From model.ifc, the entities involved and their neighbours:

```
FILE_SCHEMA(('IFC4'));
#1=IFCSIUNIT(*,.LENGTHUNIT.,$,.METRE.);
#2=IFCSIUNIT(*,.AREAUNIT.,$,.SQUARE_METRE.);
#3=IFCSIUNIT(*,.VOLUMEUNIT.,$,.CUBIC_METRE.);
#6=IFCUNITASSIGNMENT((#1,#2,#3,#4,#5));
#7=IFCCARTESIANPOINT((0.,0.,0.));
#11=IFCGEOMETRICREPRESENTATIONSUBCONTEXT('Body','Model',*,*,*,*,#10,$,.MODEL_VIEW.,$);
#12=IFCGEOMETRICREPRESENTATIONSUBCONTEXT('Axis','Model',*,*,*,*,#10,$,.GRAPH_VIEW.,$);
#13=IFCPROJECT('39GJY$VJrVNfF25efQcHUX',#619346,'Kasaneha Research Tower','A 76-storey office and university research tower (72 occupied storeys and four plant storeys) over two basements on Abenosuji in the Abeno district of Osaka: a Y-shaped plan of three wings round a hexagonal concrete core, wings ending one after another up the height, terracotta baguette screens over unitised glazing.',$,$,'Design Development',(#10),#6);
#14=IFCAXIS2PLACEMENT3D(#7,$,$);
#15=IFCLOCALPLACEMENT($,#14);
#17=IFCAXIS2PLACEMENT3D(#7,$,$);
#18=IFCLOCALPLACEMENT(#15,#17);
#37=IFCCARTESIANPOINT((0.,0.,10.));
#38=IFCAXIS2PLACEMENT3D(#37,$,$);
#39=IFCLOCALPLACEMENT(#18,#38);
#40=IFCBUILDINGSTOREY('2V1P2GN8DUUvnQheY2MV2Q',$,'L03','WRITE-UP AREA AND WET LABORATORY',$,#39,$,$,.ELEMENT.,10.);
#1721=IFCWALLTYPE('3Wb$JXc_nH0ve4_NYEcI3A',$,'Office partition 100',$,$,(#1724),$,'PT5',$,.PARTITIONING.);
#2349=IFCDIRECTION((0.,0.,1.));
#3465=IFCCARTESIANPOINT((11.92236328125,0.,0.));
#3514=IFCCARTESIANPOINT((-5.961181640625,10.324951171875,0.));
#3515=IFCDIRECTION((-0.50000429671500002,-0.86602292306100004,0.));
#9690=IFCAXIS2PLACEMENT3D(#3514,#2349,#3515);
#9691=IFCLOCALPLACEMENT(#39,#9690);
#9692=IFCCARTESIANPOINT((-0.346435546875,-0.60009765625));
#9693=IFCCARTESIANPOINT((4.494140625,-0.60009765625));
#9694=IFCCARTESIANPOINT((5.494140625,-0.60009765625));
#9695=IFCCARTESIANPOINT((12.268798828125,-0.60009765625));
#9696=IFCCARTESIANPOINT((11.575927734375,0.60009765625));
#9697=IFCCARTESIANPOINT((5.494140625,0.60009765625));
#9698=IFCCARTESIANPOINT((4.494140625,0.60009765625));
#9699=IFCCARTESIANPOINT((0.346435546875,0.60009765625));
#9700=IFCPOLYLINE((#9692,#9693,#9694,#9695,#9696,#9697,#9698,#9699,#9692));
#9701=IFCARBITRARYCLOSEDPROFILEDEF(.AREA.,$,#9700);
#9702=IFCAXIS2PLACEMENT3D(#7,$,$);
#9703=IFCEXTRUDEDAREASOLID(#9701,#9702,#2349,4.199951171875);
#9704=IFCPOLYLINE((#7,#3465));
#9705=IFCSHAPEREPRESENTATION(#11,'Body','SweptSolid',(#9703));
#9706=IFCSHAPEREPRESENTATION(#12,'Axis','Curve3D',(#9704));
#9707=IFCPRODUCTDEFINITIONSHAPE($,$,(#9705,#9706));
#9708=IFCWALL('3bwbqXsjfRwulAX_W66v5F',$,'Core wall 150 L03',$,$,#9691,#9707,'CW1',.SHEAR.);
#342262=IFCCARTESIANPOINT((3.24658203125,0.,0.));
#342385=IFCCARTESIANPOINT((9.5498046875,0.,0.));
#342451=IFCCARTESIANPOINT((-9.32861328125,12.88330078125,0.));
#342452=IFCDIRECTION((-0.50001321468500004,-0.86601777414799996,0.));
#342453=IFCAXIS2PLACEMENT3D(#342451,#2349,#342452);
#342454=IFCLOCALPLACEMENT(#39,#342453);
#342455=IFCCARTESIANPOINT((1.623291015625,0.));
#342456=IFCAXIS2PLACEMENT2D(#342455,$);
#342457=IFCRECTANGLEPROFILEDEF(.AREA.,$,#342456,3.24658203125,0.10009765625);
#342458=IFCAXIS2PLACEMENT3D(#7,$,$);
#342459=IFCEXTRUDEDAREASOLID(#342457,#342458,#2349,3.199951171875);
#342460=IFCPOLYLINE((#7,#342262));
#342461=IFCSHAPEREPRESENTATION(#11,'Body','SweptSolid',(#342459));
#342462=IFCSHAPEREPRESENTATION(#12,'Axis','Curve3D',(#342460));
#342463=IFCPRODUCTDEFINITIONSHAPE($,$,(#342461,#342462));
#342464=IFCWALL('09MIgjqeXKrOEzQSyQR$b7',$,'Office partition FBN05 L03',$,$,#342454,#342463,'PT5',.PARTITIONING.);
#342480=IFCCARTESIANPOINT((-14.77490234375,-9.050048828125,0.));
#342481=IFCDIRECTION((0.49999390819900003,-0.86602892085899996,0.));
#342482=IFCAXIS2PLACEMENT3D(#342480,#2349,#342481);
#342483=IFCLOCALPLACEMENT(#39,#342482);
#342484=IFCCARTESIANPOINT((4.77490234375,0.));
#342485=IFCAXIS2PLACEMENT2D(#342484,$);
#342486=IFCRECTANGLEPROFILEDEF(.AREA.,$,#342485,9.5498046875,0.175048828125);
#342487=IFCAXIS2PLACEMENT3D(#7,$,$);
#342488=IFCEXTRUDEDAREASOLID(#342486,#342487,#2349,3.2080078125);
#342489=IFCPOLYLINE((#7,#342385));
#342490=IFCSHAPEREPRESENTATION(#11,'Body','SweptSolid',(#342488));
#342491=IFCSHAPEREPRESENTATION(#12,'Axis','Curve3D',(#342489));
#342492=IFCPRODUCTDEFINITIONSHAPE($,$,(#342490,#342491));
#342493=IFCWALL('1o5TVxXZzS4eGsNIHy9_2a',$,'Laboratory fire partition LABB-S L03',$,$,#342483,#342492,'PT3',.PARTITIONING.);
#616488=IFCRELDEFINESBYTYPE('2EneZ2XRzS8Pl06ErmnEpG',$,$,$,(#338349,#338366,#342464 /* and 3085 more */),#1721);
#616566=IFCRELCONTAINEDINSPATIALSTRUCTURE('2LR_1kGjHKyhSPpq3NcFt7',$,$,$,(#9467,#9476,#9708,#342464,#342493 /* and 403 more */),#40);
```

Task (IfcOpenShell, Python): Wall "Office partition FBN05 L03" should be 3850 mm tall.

```python
import ifcopenshell
import ifcopenshell.geom
import ifcopenshell.util.representation
import ifcopenshell.util.shape
import ifcopenshell.util.unit

model = ifcopenshell.open("model.ifc")
unit_scale = ifcopenshell.util.unit.calculate_unit_scale(model)
settings = ifcopenshell.geom.settings()


def volume(element):
    """Net volume in cubic metres, openings subtracted."""
    shape = ifcopenshell.geom.create_shape(settings, element)
    return ifcopenshell.util.shape.get_volume(shape.geometry)


wall = model.by_guid("09MIgjqeXKrOEzQSyQR$b7")
before = volume(wall)

body = ifcopenshell.util.representation.get_representation(wall, "Model", "Body")
solid = body.Items[0]
old_height = solid.Depth
solid.Depth = 3.85 / unit_scale
after = volume(wall)

print(f"height {old_height:g} -> {solid.Depth:g}, volume {before:.3f} -> {after:.3f} m3")

model.write("model_edited.ifc")
```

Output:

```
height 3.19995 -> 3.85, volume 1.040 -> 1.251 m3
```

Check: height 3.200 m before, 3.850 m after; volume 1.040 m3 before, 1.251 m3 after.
